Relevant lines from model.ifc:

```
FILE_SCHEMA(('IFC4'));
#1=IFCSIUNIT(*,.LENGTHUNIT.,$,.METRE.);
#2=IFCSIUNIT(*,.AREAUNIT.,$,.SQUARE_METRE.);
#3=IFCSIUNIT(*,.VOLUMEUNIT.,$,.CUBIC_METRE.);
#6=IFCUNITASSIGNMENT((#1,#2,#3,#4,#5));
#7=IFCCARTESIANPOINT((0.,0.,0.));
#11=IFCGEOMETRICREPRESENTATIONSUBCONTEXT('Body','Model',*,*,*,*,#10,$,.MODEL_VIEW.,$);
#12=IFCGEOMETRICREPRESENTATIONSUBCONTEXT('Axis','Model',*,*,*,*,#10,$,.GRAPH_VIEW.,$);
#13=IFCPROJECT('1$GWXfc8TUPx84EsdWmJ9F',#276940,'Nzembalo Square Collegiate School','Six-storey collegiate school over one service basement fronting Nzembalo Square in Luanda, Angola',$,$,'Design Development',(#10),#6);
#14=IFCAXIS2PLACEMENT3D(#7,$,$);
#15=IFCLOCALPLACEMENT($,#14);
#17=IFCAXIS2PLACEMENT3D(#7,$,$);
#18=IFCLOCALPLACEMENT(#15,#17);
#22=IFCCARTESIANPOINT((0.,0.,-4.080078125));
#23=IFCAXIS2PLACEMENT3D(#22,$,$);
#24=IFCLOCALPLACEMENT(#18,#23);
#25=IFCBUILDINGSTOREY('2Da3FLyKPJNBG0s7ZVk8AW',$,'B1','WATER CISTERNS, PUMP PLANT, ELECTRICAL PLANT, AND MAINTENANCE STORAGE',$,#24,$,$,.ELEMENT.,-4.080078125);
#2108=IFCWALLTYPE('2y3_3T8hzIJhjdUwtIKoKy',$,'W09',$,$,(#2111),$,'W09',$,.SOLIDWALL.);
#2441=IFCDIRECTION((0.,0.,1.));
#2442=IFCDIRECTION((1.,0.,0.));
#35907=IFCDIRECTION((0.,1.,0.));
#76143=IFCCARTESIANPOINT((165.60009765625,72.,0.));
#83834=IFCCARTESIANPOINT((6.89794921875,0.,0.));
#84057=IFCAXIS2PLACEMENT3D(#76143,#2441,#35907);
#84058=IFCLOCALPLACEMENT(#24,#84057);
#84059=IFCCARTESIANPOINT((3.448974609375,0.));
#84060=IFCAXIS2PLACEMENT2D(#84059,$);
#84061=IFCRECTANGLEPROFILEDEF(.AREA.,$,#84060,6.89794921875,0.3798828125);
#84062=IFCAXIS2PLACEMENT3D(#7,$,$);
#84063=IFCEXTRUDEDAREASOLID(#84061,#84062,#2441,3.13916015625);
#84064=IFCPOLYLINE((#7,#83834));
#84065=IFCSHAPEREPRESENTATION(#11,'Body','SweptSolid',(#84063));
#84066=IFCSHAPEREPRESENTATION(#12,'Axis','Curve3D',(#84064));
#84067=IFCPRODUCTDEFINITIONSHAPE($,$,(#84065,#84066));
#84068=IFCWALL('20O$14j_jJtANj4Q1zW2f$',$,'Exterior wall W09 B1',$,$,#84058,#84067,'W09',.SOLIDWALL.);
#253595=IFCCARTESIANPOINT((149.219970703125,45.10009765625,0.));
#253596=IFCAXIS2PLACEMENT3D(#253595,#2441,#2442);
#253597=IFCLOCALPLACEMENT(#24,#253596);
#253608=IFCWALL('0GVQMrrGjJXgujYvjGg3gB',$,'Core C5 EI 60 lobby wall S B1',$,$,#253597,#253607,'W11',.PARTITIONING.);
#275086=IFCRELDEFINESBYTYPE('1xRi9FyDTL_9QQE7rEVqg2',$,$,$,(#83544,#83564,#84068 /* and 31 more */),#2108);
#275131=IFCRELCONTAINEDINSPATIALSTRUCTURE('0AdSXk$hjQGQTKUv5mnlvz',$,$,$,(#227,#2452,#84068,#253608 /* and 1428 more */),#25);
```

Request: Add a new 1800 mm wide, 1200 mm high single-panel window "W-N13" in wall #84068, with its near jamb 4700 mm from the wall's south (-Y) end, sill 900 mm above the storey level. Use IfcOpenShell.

```python
import numpy as np
import ifcopenshell
import ifcopenshell.api.feature
import ifcopenshell.api.geometry
import ifcopenshell.api.root
import ifcopenshell.api.spatial
import ifcopenshell.geom
import ifcopenshell.util.element
import ifcopenshell.util.placement
import ifcopenshell.util.representation
import ifcopenshell.util.shape
import ifcopenshell.util.unit

model = ifcopenshell.open("model.ifc")
unit_scale = ifcopenshell.util.unit.calculate_unit_scale(model)
settings = ifcopenshell.geom.settings()


def volume(element):
    """Net volume in cubic metres, openings subtracted."""
    shape = ifcopenshell.geom.create_shape(settings, element)
    return ifcopenshell.util.shape.get_volume(shape.geometry)


wall = model.by_guid("20O$14j_jJtANj4Q1zW2f$")
storey = ifcopenshell.util.element.get_container(wall, ifc_class="IfcBuildingStorey")
context = ifcopenshell.util.representation.get_context(model, "Model", "Body", "MODEL_VIEW")
before = volume(wall)

width, height, from_end, sill = 1.8, 1.2, 4.7, 0.9  # metres

# The wall runs along its own X axis, and the end named is its -X end.
wall_shape = ifcopenshell.geom.create_shape(settings, wall)
x, y, z = ifcopenshell.util.shape.get_vertices(wall_shape.geometry).T
start = x.min() + from_end
face, thickness = float(y.min()), float(y.max() - y.min())
wall_matrix = ifcopenshell.util.placement.get_local_placement(wall.ObjectPlacement)
level = ifcopenshell.util.placement.get_local_placement(storey.ObjectPlacement)[2, 3]


def in_wall(x, y):
    """Placement at x, y metres in the wall's axes, at sill height."""
    matrix = wall_matrix.copy()
    matrix[:, 3] = wall_matrix @ np.array([x / unit_scale, y / unit_scale, 0.0, 1.0])
    matrix[2, 3] = level + sill / unit_scale
    return matrix


# Opening: a box that overshoots both wall faces by 50 mm.
opening = ifcopenshell.api.root.create_entity(model, ifc_class="IfcOpeningElement", predefined_type="OPENING")
box = ifcopenshell.api.geometry.add_wall_representation(
    model, context=context, length=width, height=height, thickness=thickness + 0.1
)
ifcopenshell.api.geometry.assign_representation(model, product=opening, representation=box)
ifcopenshell.api.geometry.edit_object_placement(model, product=opening, matrix=in_wall(start, face - 0.05), is_si=False)
ifcopenshell.api.feature.add_feature(model, feature=opening, element=wall)

window = ifcopenshell.api.root.create_entity(model, ifc_class="IfcWindow", name="W-N13", predefined_type="WINDOW")
window.OverallWidth, window.OverallHeight = width / unit_scale, height / unit_scale
window.PartitioningType = "SINGLE_PANEL"
body = ifcopenshell.api.geometry.add_window_representation(
    model,
    context=context,
    overall_width=window.OverallWidth,
    overall_height=window.OverallHeight,
    partition_type="SINGLE_PANEL",
)
ifcopenshell.api.geometry.assign_representation(model, product=window, representation=body)
ifcopenshell.api.spatial.assign_container(model, products=[window], relating_structure=storey)
ifcopenshell.api.feature.add_filling(model, opening=opening, element=window)

# Centre the window in the wall's thickness.
ifcopenshell.api.geometry.edit_object_placement(model, product=window, matrix=in_wall(start, face), is_si=False)
window_shape = ifcopenshell.geom.create_shape(settings, window)
depth = ifcopenshell.util.shape.get_vertices(window_shape.geometry)[:, 1]
offset = face + thickness / 2 - (depth.min() + depth.max()) / 2
ifcopenshell.api.geometry.edit_object_placement(model, product=window, matrix=in_wall(start, offset), is_si=False)

after = volume(wall)

print(f"wall volume {before:.3f} -> {after:.3f} m3")

model.write("model_updated.ifc")
```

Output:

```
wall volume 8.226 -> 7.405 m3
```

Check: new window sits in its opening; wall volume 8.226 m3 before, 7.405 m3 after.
